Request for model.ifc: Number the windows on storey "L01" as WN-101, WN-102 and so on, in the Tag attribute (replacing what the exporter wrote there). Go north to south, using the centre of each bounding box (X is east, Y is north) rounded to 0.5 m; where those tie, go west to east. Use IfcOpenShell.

First a look at what the model holds.

```python
import ifcopenshell
import ifcopenshell.util.element
import ifcopenshell.util.placement

model = ifcopenshell.open("model.ifc")
print(model.schema)
storey = next(s for s in model.by_type("IfcBuildingStorey") if s.Name == "L01")
windows = [e for e in ifcopenshell.util.element.get_decomposition(storey) if e.is_a("IfcWindow")]
for e in sorted(windows, key=lambda e: e.id()):
    origin = ifcopenshell.util.placement.get_local_placement(e.ObjectPlacement)[:3, 3]
    print(e.id(), e.Tag, e.Name, origin.round(2) + 0.0, sep=" | ")
```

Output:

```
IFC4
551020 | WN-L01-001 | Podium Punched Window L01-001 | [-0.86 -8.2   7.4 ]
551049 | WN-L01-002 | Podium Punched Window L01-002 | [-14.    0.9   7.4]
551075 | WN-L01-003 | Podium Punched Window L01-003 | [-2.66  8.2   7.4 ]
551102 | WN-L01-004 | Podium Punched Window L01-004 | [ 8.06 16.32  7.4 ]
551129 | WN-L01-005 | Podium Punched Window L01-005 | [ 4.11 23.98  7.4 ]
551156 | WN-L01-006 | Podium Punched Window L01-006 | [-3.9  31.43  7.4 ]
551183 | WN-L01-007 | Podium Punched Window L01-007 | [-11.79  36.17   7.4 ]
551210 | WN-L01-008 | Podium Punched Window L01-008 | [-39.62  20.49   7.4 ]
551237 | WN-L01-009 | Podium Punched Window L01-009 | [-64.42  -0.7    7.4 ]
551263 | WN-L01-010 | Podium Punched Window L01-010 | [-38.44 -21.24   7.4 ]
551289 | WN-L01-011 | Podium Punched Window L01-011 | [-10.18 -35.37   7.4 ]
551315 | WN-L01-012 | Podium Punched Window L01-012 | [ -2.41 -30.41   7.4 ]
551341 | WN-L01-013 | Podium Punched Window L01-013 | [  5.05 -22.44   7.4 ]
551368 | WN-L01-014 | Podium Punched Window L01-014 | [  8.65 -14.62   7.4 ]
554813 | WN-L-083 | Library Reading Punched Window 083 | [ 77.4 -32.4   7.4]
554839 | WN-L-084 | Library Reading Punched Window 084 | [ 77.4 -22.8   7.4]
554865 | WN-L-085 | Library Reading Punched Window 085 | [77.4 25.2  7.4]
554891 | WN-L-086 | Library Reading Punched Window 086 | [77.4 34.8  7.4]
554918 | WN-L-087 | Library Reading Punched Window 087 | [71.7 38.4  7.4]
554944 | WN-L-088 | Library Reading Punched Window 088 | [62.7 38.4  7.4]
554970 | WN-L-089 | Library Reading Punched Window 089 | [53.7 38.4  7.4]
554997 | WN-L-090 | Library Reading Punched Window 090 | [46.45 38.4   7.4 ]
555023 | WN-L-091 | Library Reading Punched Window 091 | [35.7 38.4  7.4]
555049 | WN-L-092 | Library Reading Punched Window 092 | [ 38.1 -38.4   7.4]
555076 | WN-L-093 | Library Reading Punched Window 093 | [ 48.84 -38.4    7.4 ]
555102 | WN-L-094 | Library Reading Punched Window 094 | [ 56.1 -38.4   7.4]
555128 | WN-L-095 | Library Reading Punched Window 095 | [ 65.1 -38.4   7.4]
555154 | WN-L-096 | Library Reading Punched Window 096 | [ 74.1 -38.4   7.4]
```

```python
import ifcopenshell
import ifcopenshell.geom
import ifcopenshell.util.element
import ifcopenshell.util.shape

model = ifcopenshell.open("model.ifc")
settings = ifcopenshell.geom.settings()
settings.set("use-world-coords", True)


def centre(element):
    shape = ifcopenshell.geom.create_shape(settings, element)
    return ifcopenshell.util.shape.get_bbox_centroid(shape.geometry)


storey = next(s for s in model.by_type("IfcBuildingStorey") if s.Name == "L01")
windows = [e for e in ifcopenshell.util.element.get_decomposition(storey) if e.is_a("IfcWindow")]

# Insertion points can sit at a corner or the storey origin, so sort by the geometry (in metres).
centres = {e: centre(e) for e in windows}
windows.sort(key=lambda e: (-round(centres[e][1] / 0.5), centres[e][0]))

for i, e in enumerate(windows, start=1):
    number = f"WN-1{i:02d}"
    e.Tag = number
    print(e.id(), number)

model.write("model-out.ifc")
```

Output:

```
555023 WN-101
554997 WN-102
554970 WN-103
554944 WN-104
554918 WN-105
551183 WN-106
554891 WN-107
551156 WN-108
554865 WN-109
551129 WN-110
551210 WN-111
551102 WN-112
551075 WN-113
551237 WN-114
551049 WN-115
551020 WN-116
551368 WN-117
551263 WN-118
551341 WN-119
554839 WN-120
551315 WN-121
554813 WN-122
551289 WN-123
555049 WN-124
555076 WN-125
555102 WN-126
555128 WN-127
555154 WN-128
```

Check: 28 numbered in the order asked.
